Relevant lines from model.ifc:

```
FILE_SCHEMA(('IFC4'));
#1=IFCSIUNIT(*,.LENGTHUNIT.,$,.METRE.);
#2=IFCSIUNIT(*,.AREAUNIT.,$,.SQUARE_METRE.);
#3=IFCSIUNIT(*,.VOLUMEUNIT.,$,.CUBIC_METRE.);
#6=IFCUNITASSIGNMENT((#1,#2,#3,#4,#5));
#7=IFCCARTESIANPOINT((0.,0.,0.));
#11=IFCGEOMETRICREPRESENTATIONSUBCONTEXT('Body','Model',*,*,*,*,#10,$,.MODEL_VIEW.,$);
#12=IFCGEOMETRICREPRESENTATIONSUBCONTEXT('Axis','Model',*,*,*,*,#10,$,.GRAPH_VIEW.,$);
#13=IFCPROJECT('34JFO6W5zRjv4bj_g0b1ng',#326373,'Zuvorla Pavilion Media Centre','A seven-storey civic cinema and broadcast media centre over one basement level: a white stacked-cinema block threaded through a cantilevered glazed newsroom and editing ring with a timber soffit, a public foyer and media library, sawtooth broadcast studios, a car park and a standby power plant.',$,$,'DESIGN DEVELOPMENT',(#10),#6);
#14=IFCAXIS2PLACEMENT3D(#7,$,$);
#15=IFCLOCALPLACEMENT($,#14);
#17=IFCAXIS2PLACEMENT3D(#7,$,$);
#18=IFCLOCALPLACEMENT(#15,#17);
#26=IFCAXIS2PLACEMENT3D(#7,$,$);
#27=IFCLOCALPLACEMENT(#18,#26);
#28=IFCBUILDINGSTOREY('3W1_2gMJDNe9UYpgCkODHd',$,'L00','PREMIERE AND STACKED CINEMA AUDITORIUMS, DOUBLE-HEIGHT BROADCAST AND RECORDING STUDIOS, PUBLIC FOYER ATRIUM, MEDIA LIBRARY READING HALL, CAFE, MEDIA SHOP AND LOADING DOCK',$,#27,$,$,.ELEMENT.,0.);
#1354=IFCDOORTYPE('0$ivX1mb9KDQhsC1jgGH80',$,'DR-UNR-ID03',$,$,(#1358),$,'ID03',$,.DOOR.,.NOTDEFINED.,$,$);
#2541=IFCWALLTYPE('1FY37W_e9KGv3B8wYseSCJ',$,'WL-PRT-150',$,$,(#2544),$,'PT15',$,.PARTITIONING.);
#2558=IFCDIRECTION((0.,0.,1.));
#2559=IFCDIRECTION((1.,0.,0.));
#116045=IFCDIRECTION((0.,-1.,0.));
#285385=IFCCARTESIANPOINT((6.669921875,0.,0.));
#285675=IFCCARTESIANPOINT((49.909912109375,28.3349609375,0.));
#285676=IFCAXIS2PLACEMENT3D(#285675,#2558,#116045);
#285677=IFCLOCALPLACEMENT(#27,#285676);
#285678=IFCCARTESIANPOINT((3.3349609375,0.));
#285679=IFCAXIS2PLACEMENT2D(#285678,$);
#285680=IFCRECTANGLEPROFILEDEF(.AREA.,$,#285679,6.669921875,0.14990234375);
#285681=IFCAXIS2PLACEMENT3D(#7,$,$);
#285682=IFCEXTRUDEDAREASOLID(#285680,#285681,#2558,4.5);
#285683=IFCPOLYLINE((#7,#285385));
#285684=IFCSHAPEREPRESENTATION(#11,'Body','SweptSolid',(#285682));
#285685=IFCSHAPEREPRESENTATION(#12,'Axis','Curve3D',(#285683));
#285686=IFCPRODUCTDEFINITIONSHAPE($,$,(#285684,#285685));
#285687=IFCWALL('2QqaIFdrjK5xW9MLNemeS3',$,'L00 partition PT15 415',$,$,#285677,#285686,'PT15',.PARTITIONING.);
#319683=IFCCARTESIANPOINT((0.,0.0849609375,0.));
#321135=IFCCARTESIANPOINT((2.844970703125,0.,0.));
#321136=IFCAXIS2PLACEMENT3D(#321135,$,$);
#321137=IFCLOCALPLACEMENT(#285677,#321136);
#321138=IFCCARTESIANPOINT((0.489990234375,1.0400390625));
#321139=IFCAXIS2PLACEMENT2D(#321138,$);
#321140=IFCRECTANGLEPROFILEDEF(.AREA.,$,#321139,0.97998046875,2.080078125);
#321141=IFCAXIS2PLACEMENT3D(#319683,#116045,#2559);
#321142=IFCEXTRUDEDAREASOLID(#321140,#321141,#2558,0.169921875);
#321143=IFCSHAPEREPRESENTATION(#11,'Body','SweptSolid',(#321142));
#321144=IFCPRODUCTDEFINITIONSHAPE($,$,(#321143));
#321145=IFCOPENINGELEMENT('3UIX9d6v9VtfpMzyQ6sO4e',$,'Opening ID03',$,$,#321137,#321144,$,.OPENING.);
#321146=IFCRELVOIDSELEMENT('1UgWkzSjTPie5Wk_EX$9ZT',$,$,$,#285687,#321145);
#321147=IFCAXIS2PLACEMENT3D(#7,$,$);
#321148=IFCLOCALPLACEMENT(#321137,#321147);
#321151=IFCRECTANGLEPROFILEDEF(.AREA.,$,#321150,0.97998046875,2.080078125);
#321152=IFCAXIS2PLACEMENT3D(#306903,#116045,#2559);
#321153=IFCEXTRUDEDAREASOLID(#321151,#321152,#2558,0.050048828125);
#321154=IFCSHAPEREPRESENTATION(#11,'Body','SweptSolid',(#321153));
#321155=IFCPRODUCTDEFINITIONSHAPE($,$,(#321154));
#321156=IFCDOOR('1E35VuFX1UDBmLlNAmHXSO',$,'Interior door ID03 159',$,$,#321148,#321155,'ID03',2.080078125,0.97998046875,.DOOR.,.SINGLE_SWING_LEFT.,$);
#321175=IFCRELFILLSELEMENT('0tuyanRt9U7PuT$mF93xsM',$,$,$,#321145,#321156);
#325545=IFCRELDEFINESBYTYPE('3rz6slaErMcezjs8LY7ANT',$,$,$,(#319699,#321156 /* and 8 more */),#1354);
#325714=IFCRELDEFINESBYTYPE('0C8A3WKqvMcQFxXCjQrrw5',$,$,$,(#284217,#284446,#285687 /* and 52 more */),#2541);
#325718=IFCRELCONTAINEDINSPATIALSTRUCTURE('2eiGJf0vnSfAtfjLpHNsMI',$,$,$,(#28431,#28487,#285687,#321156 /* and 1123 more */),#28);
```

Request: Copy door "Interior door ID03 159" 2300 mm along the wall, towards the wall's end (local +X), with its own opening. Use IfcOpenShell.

```python
import ifcopenshell
import ifcopenshell.api.feature
import ifcopenshell.api.geometry
import ifcopenshell.api.root
import ifcopenshell.geom
import ifcopenshell.util.element
import ifcopenshell.util.placement
import ifcopenshell.util.shape

model = ifcopenshell.open("model.ifc")
settings = ifcopenshell.geom.settings()


def volume(element):
    """Net volume in cubic metres, openings subtracted."""
    shape = ifcopenshell.geom.create_shape(settings, element)
    return ifcopenshell.util.shape.get_volume(shape.geometry)


door = model.by_guid("1E35VuFX1UDBmLlNAmHXSO")
opening = door.FillsVoids[0].RelatingOpeningElement
wall = opening.VoidsElements[0].RelatingBuildingElement
before = volume(wall)
shift = ifcopenshell.util.placement.get_local_placement(wall.ObjectPlacement)[:3, 0] * 2.3

# copy_class copies the void relationship, type, container and properties, but no geometry.
new_opening = ifcopenshell.api.root.copy_class(model, product=opening)
new_opening.Representation = ifcopenshell.util.element.copy_deep(
    model, opening.Representation, exclude=["IfcGeometricRepresentationContext", "IfcRepresentationMap"]
)
new_door = ifcopenshell.api.root.copy_class(model, product=door)
new_door.Representation = ifcopenshell.util.element.copy_deep(
    model, door.Representation, exclude=["IfcGeometricRepresentationContext", "IfcRepresentationMap"]
)
new_door.Tag = None
ifcopenshell.api.feature.add_filling(model, opening=new_opening, element=new_door)

for old, new in ((opening, new_opening), (door, new_door)):
    matrix = ifcopenshell.util.placement.get_local_placement(old.ObjectPlacement)
    matrix[:3, 3] += shift
    ifcopenshell.api.geometry.edit_object_placement(model, product=new, matrix=matrix, is_si=False)

after = volume(wall)

print(f"wall volume {before:.3f} -> {after:.3f} m3")

model.write("model_edited.ifc")
```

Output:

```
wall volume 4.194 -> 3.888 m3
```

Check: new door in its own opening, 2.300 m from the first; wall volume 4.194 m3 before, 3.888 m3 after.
